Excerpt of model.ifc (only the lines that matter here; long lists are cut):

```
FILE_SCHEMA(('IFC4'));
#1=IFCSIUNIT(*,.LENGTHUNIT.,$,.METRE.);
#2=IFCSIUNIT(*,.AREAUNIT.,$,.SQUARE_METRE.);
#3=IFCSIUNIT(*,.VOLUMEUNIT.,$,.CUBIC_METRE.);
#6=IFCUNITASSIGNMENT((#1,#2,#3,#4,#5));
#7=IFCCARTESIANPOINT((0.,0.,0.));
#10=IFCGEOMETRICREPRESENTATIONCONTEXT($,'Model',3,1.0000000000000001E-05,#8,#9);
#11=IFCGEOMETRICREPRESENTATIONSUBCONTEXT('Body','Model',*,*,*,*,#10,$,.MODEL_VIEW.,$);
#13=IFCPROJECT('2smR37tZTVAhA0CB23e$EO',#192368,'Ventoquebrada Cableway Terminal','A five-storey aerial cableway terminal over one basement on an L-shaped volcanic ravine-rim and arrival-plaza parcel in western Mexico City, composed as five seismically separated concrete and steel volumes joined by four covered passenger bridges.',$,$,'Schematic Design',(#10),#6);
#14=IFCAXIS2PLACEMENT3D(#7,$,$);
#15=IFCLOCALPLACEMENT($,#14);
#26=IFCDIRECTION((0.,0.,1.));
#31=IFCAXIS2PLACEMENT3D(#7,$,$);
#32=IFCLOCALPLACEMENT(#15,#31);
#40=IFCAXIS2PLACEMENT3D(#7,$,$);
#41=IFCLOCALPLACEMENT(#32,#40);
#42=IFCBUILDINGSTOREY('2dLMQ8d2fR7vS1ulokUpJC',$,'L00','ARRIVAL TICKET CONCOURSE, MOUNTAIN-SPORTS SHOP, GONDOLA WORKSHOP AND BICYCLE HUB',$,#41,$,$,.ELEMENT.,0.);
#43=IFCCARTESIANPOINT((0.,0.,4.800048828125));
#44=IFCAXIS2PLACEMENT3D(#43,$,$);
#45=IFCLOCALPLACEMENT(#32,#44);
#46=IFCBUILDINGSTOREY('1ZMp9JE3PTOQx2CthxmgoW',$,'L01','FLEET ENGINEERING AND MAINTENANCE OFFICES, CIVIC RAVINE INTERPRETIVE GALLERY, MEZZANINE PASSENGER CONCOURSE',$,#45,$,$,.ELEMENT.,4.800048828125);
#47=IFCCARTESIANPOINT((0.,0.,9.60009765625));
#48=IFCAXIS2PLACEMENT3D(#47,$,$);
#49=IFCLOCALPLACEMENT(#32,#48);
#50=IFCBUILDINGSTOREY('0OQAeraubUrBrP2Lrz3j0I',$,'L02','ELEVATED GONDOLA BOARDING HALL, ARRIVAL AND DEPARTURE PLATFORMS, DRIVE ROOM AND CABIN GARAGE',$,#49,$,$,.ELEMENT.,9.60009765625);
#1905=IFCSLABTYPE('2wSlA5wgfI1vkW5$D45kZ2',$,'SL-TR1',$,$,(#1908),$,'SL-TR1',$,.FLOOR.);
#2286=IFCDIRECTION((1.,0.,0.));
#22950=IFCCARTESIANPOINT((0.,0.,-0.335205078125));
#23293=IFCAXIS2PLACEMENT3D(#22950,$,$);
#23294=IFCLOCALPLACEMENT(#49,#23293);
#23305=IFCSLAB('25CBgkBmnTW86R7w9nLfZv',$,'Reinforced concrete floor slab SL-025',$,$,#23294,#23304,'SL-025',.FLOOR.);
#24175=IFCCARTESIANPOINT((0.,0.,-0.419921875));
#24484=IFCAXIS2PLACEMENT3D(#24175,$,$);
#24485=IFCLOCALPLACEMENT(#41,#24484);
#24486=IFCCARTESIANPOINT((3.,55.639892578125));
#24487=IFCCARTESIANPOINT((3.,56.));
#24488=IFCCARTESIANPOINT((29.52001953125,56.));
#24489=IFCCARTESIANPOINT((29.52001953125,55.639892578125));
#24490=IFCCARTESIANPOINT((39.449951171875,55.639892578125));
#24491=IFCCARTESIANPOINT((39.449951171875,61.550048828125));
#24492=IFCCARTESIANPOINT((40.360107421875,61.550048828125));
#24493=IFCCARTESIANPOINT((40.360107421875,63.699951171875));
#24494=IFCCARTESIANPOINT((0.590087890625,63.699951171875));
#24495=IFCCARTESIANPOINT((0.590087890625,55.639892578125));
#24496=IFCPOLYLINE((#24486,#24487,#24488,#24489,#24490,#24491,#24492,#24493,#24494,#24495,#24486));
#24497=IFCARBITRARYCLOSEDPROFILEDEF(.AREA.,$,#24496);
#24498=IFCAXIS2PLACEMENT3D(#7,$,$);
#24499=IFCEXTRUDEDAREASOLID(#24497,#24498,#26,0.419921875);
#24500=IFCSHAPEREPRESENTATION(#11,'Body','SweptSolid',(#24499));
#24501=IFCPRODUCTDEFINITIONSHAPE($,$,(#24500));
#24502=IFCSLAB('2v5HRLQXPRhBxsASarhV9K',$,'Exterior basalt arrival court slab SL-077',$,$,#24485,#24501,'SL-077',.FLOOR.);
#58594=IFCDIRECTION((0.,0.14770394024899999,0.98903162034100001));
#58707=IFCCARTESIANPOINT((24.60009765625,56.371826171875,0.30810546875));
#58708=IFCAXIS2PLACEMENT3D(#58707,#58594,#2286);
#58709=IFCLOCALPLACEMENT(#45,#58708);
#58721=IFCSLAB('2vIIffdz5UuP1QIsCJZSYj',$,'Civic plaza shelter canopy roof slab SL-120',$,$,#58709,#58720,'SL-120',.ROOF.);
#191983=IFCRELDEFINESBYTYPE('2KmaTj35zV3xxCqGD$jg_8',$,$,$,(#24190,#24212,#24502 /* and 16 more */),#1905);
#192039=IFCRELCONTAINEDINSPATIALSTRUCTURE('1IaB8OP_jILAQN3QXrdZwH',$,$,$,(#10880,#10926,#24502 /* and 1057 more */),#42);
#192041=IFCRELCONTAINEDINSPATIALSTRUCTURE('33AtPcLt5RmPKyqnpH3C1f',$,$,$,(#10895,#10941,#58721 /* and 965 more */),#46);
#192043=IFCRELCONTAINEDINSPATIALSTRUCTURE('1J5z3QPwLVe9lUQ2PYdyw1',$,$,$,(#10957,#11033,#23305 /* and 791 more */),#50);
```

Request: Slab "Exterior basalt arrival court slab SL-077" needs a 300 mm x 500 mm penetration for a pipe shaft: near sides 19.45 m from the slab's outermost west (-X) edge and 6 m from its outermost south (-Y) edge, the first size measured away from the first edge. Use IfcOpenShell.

```python
import numpy as np
import ifcopenshell
import ifcopenshell.api.feature
import ifcopenshell.api.geometry
import ifcopenshell.api.root
import ifcopenshell.geom
import ifcopenshell.util.placement
import ifcopenshell.util.representation
import ifcopenshell.util.shape
import ifcopenshell.util.unit

model = ifcopenshell.open("model.ifc")
unit_scale = ifcopenshell.util.unit.calculate_unit_scale(model)
settings = ifcopenshell.geom.settings()


def volume(element):
    """Net volume in cubic metres, openings subtracted."""
    shape = ifcopenshell.geom.create_shape(settings, element)
    return ifcopenshell.util.shape.get_volume(shape.geometry)


slab = model.by_id(24502)
before = volume(slab)

# Extent in the slab's own axes, in metres. The edges named are its -X and -Y sides.
slab_shape = ifcopenshell.geom.create_shape(settings, slab)
vertices = ifcopenshell.util.shape.get_vertices(slab_shape.geometry)
x_min, y_min, bottom = vertices.min(axis=0)
top = vertices[:, 2].max()

opening = ifcopenshell.api.root.create_entity(model, ifc_class="IfcOpeningElement", name="Pipe shaft opening", predefined_type="OPENING")
context = ifcopenshell.util.representation.get_context(model, "Model", "Body", "MODEL_VIEW")
width, depth = 0.3, 0.5
outline = [(0.0, 0.0), (width, 0.0), (width, depth), (0.0, depth), (0.0, 0.0)]
# Overshoot both faces by 50 mm so the cut is clean.
shape = ifcopenshell.api.geometry.add_slab_representation(
    model, context=context, depth=top - bottom + 0.1, polyline=outline
)
ifcopenshell.api.geometry.assign_representation(model, product=opening, representation=shape)

matrix = ifcopenshell.util.placement.get_local_placement(slab.ObjectPlacement)
matrix[:, 3] = matrix @ np.append(np.array([x_min + 19.45, y_min + 6, bottom - 0.05]) / unit_scale, 1.0)
ifcopenshell.api.geometry.edit_object_placement(model, product=opening, matrix=matrix, is_si=False)
ifcopenshell.api.feature.add_feature(model, feature=opening, element=slab)

after = volume(slab)

print(f"slab volume {before:.3f} -> {after:.3f} m3")

model.write("model-out.ifc")
```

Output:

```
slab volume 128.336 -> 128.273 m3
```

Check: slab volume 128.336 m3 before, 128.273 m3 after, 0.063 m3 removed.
